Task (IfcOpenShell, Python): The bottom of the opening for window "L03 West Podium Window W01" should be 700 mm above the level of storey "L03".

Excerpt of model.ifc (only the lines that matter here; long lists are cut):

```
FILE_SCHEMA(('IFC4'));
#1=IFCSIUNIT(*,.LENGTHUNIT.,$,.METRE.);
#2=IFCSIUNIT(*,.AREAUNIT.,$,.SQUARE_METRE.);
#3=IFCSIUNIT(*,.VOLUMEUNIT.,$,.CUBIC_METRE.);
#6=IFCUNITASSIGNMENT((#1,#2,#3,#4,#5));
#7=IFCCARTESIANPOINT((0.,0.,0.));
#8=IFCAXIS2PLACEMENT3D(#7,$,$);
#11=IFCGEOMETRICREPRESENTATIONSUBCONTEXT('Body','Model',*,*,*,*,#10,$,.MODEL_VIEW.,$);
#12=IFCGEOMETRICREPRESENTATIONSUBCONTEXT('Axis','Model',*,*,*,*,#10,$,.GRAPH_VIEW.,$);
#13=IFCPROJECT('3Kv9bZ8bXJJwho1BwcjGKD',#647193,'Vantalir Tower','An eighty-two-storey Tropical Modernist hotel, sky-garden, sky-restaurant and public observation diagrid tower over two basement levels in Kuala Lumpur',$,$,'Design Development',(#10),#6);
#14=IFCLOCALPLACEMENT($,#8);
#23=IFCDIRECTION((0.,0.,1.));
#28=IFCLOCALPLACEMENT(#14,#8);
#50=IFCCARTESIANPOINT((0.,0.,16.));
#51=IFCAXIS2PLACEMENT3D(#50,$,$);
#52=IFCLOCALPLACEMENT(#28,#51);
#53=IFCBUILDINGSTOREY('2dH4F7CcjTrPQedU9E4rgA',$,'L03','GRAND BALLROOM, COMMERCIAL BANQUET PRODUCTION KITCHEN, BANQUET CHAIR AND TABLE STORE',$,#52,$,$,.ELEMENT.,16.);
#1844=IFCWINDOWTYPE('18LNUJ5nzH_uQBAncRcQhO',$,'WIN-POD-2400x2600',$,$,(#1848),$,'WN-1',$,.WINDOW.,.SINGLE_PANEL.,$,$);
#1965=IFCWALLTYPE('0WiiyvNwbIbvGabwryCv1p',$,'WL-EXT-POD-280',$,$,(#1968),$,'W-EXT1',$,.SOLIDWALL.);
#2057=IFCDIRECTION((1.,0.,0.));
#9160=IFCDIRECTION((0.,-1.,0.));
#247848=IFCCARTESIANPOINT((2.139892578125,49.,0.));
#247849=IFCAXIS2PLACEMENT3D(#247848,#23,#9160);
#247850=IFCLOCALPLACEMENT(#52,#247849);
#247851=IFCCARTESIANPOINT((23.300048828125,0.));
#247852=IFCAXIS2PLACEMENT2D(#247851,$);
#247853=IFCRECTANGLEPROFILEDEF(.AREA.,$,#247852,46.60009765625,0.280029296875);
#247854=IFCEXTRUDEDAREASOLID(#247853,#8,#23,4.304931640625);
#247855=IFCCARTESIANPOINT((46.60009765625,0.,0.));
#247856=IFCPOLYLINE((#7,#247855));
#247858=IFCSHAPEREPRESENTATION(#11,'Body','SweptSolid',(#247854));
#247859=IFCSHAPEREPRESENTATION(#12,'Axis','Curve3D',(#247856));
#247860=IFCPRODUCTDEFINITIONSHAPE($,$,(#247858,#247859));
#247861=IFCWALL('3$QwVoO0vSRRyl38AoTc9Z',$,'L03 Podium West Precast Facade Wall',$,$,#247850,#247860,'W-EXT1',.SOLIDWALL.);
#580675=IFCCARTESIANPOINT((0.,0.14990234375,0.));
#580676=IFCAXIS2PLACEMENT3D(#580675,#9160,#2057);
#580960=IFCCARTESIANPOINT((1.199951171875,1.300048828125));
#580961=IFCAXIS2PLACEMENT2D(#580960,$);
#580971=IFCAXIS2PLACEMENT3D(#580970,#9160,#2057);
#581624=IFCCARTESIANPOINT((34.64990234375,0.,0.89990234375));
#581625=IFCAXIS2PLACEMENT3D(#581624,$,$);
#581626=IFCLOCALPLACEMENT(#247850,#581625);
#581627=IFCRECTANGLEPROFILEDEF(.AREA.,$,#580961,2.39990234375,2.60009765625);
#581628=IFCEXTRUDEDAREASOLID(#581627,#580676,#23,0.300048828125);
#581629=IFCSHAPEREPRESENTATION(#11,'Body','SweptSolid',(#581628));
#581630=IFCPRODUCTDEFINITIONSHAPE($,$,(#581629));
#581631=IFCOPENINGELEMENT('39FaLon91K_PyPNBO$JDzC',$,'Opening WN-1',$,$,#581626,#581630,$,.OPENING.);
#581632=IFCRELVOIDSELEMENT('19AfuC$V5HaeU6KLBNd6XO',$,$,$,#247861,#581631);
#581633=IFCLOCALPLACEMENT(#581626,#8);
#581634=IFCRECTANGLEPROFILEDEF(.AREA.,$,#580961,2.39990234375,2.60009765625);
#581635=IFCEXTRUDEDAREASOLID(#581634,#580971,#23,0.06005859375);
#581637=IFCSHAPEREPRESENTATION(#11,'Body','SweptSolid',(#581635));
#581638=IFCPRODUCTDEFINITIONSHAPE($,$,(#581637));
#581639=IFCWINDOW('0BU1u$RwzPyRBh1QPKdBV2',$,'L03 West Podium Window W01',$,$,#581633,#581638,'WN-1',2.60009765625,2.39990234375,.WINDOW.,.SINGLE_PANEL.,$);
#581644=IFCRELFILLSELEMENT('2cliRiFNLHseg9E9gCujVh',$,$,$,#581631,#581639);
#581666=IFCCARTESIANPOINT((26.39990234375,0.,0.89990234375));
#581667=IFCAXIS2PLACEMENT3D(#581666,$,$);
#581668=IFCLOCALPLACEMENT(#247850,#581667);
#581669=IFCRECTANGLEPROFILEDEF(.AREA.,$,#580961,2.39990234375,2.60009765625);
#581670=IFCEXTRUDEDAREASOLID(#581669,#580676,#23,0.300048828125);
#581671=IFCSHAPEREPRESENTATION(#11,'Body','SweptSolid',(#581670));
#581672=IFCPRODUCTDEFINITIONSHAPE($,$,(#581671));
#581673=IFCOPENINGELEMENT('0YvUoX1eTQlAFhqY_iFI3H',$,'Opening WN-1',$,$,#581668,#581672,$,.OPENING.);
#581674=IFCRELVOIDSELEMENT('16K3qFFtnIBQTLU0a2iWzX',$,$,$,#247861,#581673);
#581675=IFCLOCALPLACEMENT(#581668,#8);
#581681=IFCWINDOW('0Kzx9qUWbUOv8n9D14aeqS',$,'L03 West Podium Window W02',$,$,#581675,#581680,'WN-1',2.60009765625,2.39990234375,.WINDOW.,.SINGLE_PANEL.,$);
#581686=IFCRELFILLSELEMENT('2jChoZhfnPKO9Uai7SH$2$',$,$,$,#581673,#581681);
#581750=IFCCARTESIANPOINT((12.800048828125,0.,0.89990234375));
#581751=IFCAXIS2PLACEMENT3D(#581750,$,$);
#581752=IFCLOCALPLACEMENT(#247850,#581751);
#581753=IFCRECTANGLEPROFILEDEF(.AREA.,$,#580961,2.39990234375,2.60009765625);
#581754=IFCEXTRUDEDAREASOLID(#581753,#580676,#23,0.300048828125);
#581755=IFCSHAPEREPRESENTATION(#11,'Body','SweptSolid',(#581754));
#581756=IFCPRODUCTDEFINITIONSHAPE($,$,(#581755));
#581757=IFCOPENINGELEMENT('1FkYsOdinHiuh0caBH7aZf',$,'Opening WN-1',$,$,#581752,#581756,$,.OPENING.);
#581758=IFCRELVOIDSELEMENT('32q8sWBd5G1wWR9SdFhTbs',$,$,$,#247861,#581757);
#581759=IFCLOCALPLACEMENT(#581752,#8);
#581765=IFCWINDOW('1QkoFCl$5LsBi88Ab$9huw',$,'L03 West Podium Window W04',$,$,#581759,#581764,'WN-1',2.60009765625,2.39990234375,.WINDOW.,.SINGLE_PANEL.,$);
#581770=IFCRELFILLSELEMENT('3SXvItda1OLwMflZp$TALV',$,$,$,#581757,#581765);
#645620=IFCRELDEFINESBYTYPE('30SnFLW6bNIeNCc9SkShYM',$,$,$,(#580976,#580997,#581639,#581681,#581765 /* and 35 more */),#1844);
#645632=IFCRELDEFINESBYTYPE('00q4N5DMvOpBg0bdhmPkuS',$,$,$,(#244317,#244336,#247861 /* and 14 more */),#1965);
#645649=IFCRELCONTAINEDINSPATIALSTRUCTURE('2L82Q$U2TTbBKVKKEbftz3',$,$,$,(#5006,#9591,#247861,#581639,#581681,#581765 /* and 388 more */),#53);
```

```python
import numpy as np
import ifcopenshell
import ifcopenshell.api.geometry
import ifcopenshell.geom
import ifcopenshell.util.element
import ifcopenshell.util.placement
import ifcopenshell.util.shape
import ifcopenshell.util.unit

model = ifcopenshell.open("model.ifc")
unit_scale = ifcopenshell.util.unit.calculate_unit_scale(model)

window = model.by_guid("0BU1u$RwzPyRBh1QPKdBV2")
opening = window.FillsVoids[0].RelatingOpeningElement
storey = ifcopenshell.util.element.get_container(window, ifc_class="IfcBuildingStorey")
level = ifcopenshell.util.placement.get_local_placement(storey.ObjectPlacement)[2, 3]

# The opening's origin need not be at the sill, so measure its lowest point.
shape = ifcopenshell.geom.create_shape(ifcopenshell.geom.settings(), opening)
bottom = ifcopenshell.util.shape.get_shape_bottom_elevation(shape, shape.geometry) / unit_scale
dz = level + 0.7 / unit_scale - bottom

shift = np.array([0.0, 0.0, dz])
# The window is placed relative to its opening, so it follows when the opening moves.
matrix = ifcopenshell.util.placement.get_local_placement(opening.ObjectPlacement)
matrix[:3, 3] += shift
ifcopenshell.api.geometry.edit_object_placement(
    model, product=opening, matrix=matrix, is_si=False, should_transform_children=True
)

print(f"moved by {dz * unit_scale:+.3f} m")

model.write("model_edited.ifc")
```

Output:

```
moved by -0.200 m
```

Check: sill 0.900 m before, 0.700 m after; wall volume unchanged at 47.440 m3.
